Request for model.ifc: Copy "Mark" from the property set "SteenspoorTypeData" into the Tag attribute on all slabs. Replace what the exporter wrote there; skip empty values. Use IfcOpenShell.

First a look at what the model holds.

```python
import ifcopenshell
import ifcopenshell.util.element

model = ifcopenshell.open("model.ifc")
print(model.schema)
slabs = model.by_type("IfcSlab")
print(len(slabs), "slabs")
for e in slabs[:8]:
    source = ifcopenshell.util.element.get_pset(e, "SteenspoorTypeData", "Mark")
    target = e.Tag
    print(e.id(), repr(source), repr(target), sep=" | ")
```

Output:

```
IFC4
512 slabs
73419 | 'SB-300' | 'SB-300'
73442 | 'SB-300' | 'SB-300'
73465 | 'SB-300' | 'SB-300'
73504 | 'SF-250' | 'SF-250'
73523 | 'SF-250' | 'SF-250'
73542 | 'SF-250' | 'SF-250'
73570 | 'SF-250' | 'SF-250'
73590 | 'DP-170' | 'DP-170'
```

```python
import ifcopenshell
import ifcopenshell.util.element

model = ifcopenshell.open("model.ifc")

count = 0
for e in model.by_type("IfcSlab"):
    value = ifcopenshell.util.element.get_pset(e, "SteenspoorTypeData", "Mark")
    current = e.Tag
    if not value or not value.strip() or current == value:
        continue
    e.Tag = value
    count += 1

print(count, "slabs updated")

model.write("model_updated.ifc")
```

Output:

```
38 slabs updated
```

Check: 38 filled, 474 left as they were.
